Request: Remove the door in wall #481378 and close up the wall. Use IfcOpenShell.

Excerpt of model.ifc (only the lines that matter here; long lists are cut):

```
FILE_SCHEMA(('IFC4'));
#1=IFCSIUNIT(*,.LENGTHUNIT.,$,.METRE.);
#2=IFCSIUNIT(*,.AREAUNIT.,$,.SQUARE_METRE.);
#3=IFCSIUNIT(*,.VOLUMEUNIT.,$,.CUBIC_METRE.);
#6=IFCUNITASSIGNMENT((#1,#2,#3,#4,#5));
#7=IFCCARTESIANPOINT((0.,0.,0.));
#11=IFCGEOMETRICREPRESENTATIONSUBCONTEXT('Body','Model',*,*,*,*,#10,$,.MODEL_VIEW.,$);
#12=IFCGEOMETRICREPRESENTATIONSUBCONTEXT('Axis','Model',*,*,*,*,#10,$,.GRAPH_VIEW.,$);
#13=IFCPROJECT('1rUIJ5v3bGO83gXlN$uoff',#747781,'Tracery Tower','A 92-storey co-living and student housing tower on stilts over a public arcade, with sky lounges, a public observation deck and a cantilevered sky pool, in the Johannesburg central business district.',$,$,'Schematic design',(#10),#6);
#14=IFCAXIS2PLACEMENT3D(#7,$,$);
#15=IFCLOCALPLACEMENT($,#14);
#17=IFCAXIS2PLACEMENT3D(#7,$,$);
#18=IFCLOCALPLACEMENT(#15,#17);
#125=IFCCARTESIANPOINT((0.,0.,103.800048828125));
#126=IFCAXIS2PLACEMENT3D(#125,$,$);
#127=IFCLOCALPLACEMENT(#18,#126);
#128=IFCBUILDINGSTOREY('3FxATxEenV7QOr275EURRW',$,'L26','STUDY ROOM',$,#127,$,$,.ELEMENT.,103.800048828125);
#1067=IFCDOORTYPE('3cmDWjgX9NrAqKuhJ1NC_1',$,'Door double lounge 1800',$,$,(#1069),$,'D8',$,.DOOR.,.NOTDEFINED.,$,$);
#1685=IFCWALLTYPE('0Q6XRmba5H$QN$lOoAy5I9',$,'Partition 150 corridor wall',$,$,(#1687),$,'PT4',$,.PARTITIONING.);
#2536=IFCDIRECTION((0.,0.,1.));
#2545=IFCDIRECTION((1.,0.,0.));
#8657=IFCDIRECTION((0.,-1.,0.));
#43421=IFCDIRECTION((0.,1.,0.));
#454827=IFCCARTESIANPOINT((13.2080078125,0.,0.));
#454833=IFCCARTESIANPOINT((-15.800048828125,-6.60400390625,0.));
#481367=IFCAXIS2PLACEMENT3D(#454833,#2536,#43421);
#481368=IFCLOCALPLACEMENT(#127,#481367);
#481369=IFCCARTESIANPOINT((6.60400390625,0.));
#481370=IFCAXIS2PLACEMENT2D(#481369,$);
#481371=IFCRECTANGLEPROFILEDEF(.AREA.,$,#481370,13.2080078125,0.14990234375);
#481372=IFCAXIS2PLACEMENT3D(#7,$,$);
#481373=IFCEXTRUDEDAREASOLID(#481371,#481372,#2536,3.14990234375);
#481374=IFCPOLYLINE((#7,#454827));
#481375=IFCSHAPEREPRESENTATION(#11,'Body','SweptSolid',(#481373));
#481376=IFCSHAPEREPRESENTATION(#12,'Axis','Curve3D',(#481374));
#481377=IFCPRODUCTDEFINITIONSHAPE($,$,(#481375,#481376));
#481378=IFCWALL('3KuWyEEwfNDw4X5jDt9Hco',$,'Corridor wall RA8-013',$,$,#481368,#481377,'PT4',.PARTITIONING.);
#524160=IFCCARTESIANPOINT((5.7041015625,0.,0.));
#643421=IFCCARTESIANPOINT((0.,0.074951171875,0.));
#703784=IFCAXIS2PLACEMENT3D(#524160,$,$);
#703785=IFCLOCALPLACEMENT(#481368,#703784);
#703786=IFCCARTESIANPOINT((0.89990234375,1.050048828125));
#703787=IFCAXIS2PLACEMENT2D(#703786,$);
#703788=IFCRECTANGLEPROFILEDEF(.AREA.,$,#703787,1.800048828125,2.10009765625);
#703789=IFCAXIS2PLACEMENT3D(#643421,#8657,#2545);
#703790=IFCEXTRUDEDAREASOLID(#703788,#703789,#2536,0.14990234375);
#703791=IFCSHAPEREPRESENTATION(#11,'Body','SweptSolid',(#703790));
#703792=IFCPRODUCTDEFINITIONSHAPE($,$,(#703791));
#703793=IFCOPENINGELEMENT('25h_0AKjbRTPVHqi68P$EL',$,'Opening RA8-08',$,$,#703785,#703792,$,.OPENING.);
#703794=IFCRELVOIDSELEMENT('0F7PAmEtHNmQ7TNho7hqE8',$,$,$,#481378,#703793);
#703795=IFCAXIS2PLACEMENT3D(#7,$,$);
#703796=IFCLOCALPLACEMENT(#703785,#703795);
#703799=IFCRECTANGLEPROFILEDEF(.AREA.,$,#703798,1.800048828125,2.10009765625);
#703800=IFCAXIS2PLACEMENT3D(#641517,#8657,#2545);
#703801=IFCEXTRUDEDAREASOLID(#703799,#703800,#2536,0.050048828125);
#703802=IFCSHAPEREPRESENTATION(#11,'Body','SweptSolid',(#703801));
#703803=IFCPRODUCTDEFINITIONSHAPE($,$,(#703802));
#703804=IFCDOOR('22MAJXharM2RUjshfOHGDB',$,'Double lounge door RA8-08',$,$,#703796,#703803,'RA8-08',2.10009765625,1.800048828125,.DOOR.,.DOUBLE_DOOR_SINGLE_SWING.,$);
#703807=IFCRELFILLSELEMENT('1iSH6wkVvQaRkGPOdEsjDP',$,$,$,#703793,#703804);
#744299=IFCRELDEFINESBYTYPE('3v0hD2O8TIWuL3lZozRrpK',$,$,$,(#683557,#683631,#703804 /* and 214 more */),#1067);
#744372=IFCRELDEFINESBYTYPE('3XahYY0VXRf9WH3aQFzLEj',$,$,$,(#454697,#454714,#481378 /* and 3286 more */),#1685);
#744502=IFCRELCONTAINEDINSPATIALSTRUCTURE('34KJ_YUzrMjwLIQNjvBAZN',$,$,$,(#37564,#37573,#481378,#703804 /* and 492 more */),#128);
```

```python
import ifcopenshell
import ifcopenshell.api.feature
import ifcopenshell.api.root
import ifcopenshell.geom
import ifcopenshell.util.shape

model = ifcopenshell.open("model.ifc")
settings = ifcopenshell.geom.settings()


def volume(element):
    """Net volume in cubic metres, openings subtracted."""
    shape = ifcopenshell.geom.create_shape(settings, element)
    return ifcopenshell.util.shape.get_volume(shape.geometry)


door = model.by_guid("22MAJXharM2RUjshfOHGDB")
opening = door.FillsVoids[0].RelatingOpeningElement
wall = opening.VoidsElements[0].RelatingBuildingElement
before = volume(wall)

ifcopenshell.api.root.remove_product(model, product=door)
ifcopenshell.api.feature.remove_feature(model, feature=opening)

after = volume(wall)

print(f"wall volume {before:.3f} -> {after:.3f} m3")

model.write("model_rev.ifc")
```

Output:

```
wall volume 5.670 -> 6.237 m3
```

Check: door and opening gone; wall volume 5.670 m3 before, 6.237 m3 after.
